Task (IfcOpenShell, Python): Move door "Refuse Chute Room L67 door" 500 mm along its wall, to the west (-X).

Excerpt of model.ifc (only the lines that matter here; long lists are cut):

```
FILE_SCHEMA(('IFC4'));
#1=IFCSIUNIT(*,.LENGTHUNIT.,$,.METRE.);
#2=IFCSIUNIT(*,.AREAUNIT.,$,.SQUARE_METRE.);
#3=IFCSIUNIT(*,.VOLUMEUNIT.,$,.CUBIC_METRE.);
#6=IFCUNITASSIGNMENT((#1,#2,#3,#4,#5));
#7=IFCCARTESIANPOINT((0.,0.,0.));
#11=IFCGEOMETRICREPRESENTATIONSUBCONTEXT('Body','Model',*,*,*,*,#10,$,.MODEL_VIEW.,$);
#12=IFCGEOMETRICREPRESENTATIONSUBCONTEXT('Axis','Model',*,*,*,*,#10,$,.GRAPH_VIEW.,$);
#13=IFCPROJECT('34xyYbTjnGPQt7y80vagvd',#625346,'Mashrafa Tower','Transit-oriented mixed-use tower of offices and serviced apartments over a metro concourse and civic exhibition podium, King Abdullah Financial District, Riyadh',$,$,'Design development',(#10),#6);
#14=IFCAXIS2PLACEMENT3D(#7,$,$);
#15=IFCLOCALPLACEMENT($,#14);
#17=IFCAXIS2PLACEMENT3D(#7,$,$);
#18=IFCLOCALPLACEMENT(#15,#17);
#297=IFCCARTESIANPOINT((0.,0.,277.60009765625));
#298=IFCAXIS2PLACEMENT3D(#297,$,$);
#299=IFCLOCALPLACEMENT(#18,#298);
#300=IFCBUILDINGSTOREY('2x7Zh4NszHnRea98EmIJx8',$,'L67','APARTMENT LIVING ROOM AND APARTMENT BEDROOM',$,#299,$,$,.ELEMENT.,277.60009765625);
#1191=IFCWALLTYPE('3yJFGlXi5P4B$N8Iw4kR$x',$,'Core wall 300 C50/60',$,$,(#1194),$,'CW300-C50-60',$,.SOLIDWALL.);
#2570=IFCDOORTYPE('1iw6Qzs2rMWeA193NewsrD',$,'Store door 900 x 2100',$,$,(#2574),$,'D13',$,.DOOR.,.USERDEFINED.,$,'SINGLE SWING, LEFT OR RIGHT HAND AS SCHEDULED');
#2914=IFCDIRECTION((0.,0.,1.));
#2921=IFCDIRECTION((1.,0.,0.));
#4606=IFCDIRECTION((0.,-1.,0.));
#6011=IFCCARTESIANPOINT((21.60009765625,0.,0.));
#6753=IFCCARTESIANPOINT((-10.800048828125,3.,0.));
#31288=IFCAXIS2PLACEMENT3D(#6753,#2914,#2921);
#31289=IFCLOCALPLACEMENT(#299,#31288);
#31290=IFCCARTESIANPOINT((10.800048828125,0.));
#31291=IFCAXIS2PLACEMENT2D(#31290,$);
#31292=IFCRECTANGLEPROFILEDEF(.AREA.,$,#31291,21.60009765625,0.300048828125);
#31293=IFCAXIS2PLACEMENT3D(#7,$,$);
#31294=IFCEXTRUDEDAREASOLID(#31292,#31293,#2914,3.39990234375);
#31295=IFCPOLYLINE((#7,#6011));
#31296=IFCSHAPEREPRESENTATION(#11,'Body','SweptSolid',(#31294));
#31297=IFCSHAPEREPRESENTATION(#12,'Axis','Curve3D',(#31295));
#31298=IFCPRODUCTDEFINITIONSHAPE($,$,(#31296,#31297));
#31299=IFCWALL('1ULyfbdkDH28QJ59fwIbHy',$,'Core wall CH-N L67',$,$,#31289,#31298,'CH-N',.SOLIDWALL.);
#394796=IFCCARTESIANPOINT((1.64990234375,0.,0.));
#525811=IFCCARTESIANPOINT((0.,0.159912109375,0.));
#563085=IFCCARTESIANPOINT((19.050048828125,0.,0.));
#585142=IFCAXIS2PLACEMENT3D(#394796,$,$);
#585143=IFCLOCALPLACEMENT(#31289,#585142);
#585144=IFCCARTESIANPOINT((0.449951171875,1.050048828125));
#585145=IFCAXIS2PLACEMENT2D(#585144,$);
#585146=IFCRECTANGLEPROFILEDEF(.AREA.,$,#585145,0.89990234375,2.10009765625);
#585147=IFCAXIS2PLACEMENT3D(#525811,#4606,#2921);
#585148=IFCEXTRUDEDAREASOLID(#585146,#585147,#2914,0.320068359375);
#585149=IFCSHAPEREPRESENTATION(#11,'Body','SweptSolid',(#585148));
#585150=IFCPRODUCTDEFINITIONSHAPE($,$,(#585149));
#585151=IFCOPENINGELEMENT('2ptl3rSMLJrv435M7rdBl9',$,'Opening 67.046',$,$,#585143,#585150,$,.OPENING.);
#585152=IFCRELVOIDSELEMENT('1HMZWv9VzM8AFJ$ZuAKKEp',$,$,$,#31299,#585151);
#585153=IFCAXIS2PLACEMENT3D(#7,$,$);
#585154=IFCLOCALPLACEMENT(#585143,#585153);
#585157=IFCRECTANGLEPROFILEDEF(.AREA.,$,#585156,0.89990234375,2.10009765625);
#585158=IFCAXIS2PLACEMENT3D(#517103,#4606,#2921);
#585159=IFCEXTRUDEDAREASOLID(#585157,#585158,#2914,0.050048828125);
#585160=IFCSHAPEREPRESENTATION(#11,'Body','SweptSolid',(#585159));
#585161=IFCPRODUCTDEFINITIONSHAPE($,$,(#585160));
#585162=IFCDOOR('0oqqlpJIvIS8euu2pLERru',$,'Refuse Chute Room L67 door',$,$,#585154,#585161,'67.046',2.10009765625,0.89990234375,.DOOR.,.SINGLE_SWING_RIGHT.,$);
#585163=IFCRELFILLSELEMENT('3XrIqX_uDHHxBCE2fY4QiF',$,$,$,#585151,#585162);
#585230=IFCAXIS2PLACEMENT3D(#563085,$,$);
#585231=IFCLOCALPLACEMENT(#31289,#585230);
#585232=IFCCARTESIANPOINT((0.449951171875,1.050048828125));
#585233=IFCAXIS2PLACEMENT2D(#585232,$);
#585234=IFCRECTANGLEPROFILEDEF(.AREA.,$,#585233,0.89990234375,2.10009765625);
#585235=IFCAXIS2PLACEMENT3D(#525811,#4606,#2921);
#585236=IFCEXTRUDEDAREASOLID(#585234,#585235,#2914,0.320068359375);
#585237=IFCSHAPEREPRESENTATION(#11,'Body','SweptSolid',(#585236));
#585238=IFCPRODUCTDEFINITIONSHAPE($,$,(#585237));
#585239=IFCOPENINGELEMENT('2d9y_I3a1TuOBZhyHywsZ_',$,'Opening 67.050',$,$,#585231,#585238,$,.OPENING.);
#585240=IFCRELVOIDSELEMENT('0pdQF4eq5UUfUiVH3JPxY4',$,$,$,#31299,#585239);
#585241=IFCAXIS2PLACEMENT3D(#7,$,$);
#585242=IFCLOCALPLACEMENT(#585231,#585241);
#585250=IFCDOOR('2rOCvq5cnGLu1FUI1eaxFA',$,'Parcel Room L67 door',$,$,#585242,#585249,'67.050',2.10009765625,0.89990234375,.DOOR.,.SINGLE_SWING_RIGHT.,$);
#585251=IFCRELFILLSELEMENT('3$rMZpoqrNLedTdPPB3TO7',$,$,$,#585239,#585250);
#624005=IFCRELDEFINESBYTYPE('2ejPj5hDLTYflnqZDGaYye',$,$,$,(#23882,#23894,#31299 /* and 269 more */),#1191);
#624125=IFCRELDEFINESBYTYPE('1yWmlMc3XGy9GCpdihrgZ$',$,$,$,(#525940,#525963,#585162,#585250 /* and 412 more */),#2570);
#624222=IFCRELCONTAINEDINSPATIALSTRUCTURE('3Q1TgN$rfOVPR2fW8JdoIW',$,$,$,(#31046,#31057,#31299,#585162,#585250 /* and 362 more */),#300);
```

```python
import ifcopenshell
import ifcopenshell.api.geometry
import ifcopenshell.util.placement
import ifcopenshell.util.unit

model = ifcopenshell.open("model.ifc")
unit_scale = ifcopenshell.util.unit.calculate_unit_scale(model)

door = model.by_guid("0oqqlpJIvIS8euu2pLERru")
opening = door.FillsVoids[0].RelatingOpeningElement
wall = opening.VoidsElements[0].RelatingBuildingElement

wall_matrix = ifcopenshell.util.placement.get_local_placement(wall.ObjectPlacement)
shift = wall_matrix[:3, 0] * -0.5 / unit_scale
before = ifcopenshell.util.placement.get_local_placement(door.ObjectPlacement)[:3, 3].copy()

# The door is placed relative to its opening, so it follows when the opening moves.
matrix = ifcopenshell.util.placement.get_local_placement(opening.ObjectPlacement)
matrix[:3, 3] += shift
ifcopenshell.api.geometry.edit_object_placement(
    model, product=opening, matrix=matrix, is_si=False, should_transform_children=True
)

after = ifcopenshell.util.placement.get_local_placement(door.ObjectPlacement)[:3, 3]
print("door moved by", (after - before).round(3) + 0.0)

model.write("model_edited.ifc")
```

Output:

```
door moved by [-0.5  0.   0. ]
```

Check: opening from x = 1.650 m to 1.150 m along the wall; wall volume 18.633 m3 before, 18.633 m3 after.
